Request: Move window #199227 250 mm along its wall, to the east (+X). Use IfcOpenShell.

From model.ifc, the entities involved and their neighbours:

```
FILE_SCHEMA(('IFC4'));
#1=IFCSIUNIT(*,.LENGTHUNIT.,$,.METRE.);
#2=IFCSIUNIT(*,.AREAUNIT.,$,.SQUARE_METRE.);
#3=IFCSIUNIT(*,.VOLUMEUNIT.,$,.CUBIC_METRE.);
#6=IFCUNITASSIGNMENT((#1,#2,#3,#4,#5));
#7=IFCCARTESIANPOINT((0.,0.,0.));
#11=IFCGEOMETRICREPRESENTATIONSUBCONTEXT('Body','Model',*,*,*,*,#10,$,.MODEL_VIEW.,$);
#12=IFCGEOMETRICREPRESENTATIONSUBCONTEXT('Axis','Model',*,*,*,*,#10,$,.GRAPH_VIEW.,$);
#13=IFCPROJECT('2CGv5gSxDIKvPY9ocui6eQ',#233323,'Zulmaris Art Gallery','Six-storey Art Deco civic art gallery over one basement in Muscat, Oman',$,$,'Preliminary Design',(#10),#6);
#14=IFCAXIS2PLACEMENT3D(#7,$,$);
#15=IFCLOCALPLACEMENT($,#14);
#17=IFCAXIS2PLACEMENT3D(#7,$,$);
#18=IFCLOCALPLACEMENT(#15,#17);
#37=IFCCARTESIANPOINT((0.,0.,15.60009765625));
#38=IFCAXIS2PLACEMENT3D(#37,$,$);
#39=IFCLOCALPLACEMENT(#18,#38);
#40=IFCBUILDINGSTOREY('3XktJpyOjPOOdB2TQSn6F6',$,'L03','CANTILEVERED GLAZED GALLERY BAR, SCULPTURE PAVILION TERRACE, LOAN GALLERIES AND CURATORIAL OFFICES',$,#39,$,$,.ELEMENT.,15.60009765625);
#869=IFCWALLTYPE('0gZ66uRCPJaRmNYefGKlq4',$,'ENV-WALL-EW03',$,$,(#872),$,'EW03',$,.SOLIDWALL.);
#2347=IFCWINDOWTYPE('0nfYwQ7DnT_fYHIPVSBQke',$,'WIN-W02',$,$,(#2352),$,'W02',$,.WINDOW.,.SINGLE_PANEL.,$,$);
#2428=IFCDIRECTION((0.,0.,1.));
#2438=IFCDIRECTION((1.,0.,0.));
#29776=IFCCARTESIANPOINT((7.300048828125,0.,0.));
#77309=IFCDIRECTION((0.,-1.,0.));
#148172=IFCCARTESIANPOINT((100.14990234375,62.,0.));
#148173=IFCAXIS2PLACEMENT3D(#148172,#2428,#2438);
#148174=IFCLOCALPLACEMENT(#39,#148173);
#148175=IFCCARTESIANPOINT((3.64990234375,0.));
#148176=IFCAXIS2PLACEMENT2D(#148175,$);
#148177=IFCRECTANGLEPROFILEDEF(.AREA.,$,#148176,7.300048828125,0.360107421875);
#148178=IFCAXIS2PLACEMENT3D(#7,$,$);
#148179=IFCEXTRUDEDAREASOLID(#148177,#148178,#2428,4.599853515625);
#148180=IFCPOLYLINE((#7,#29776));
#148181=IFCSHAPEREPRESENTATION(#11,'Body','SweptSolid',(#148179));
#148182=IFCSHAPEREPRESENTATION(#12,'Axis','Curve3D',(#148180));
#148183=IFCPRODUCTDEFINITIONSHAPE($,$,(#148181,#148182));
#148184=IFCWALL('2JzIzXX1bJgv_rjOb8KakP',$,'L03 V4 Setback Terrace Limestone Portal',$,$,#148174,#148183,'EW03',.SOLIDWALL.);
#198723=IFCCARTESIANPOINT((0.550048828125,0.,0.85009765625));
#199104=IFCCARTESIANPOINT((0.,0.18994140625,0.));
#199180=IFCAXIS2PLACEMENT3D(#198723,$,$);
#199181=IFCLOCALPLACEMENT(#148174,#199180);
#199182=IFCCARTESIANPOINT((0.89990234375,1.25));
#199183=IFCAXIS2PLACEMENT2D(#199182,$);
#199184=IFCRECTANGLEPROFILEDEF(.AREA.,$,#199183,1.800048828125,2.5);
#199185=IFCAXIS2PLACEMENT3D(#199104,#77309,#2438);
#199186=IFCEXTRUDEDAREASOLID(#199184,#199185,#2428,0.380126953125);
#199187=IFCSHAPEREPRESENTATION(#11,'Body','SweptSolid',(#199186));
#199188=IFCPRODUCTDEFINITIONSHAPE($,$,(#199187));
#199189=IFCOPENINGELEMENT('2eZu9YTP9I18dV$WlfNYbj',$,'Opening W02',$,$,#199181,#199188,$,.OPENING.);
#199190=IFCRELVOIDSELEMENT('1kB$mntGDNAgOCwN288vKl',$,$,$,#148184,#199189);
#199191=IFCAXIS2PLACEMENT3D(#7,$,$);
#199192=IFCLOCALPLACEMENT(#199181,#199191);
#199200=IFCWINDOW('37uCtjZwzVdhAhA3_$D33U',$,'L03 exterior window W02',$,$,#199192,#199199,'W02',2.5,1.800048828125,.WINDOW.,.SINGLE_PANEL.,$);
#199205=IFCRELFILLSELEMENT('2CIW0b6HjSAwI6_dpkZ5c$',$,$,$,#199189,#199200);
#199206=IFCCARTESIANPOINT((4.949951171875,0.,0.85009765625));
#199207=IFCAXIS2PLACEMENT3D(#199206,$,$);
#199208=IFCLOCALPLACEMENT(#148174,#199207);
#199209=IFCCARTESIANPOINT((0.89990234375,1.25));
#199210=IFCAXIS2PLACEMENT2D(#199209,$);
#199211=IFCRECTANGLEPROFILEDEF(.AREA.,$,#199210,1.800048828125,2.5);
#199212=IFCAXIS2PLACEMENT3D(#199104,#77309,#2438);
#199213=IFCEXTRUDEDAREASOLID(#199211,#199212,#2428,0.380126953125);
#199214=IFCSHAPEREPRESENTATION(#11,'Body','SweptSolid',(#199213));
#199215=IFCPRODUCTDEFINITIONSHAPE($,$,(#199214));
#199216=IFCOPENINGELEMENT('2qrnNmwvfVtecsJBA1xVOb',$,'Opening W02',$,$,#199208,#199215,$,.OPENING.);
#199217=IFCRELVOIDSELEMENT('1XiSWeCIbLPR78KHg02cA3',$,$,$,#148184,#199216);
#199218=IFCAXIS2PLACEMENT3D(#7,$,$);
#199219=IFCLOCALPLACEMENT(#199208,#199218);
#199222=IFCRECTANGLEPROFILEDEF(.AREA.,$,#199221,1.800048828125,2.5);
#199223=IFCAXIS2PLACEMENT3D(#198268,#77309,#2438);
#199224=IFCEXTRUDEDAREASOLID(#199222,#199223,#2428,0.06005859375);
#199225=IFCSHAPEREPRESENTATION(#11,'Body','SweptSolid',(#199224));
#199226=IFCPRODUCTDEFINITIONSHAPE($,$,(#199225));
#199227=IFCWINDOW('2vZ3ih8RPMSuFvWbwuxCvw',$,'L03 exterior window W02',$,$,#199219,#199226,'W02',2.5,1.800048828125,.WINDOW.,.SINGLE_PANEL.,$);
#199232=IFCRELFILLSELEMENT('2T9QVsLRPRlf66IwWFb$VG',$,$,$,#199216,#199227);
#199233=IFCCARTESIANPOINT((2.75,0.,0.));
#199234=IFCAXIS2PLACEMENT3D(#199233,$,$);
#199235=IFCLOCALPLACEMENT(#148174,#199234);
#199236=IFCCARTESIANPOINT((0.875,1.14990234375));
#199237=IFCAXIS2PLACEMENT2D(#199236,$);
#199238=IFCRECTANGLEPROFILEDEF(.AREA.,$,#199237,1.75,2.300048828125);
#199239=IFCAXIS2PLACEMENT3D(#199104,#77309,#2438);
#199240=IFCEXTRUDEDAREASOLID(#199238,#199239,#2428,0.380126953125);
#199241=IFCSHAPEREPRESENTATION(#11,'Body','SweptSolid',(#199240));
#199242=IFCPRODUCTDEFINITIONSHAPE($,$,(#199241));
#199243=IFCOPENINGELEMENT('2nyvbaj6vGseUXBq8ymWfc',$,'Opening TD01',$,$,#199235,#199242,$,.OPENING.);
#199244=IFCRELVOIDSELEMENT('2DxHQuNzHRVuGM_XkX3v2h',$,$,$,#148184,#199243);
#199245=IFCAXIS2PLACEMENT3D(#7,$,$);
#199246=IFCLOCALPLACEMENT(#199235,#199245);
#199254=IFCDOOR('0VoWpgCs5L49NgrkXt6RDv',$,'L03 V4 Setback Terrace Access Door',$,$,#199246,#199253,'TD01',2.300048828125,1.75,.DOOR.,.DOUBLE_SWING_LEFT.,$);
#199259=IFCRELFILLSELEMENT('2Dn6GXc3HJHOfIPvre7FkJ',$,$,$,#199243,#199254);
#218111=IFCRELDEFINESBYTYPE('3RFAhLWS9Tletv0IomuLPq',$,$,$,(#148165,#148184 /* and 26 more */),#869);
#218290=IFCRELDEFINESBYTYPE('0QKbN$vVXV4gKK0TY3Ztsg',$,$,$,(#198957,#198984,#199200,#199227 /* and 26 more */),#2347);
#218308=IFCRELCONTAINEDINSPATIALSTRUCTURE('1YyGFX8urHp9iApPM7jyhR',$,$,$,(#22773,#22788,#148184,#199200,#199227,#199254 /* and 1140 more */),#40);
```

```python
import ifcopenshell
import ifcopenshell.api.geometry
import ifcopenshell.util.placement
import ifcopenshell.util.unit

model = ifcopenshell.open("model.ifc")
unit_scale = ifcopenshell.util.unit.calculate_unit_scale(model)

window = model.by_id(199227)
opening = window.FillsVoids[0].RelatingOpeningElement
wall = opening.VoidsElements[0].RelatingBuildingElement

wall_matrix = ifcopenshell.util.placement.get_local_placement(wall.ObjectPlacement)
shift = wall_matrix[:3, 0] * 0.25 / unit_scale
before = ifcopenshell.util.placement.get_local_placement(window.ObjectPlacement)[:3, 3].copy()

# The window is placed relative to its opening, so it follows when the opening moves.
matrix = ifcopenshell.util.placement.get_local_placement(opening.ObjectPlacement)
matrix[:3, 3] += shift
ifcopenshell.api.geometry.edit_object_placement(
    model, product=opening, matrix=matrix, is_si=False, should_transform_children=True
)

after = ifcopenshell.util.placement.get_local_placement(window.ObjectPlacement)[:3, 3]
print("window moved by", (after - before).round(3) + 0.0)

model.write("model_updated.ifc")
```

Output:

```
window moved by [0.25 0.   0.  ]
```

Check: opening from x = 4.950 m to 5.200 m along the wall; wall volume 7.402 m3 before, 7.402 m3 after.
